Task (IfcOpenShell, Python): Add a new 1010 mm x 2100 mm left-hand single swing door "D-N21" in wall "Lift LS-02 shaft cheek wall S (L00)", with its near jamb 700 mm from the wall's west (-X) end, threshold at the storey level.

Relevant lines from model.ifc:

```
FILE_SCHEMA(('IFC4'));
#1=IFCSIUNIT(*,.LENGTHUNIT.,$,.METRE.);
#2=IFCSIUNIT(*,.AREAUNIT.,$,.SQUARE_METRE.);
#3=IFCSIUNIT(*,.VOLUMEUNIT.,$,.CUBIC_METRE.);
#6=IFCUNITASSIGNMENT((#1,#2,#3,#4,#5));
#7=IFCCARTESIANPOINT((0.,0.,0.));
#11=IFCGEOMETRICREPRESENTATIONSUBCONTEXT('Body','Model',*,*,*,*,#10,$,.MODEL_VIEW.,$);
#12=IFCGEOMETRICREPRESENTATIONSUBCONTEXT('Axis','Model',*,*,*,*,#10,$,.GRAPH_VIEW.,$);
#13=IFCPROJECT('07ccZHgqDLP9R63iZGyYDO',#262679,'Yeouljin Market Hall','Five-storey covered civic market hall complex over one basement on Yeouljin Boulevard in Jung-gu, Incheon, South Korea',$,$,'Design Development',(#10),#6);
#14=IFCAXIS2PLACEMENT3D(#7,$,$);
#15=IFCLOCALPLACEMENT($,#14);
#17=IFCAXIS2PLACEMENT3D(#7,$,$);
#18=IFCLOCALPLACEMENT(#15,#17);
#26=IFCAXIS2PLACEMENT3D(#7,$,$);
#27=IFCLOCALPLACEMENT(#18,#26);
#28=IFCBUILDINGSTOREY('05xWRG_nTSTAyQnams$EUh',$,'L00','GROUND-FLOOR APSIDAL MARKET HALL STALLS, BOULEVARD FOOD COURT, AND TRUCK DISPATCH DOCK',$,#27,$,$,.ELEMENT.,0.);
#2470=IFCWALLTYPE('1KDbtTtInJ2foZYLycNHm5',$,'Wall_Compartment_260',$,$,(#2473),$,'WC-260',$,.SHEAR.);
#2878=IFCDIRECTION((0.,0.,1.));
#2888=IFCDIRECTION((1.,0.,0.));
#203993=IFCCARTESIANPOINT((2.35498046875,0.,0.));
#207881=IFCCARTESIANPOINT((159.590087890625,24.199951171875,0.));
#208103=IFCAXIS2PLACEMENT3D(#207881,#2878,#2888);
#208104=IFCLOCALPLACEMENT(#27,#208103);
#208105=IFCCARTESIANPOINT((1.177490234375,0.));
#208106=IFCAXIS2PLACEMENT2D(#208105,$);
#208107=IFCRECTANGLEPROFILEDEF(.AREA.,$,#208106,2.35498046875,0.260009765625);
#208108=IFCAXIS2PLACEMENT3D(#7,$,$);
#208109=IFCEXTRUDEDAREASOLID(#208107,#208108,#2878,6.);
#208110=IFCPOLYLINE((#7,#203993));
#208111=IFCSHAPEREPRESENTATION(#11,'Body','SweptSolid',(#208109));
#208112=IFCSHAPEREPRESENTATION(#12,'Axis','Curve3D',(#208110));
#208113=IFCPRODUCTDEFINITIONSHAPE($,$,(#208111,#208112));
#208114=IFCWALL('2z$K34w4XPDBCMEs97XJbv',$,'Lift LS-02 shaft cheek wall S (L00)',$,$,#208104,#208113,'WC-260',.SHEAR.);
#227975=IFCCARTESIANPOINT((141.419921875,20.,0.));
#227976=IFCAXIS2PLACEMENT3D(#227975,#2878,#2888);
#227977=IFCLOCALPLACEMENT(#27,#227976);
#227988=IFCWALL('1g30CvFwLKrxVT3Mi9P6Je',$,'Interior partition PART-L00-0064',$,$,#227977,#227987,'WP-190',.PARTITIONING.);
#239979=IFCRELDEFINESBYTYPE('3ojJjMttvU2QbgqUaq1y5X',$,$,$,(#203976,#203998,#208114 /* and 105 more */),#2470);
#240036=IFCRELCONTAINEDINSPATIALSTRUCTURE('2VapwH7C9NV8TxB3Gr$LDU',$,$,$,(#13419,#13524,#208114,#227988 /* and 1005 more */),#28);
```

```python
import numpy as np
import ifcopenshell
import ifcopenshell.api.feature
import ifcopenshell.api.geometry
import ifcopenshell.api.root
import ifcopenshell.api.spatial
import ifcopenshell.geom
import ifcopenshell.util.element
import ifcopenshell.util.placement
import ifcopenshell.util.representation
import ifcopenshell.util.shape
import ifcopenshell.util.unit

model = ifcopenshell.open("model.ifc")
unit_scale = ifcopenshell.util.unit.calculate_unit_scale(model)
settings = ifcopenshell.geom.settings()


def volume(element):
    """Net volume in cubic metres, openings subtracted."""
    shape = ifcopenshell.geom.create_shape(settings, element)
    return ifcopenshell.util.shape.get_volume(shape.geometry)


wall = model.by_id(208114)
storey = ifcopenshell.util.element.get_container(wall, ifc_class="IfcBuildingStorey")
context = ifcopenshell.util.representation.get_context(model, "Model", "Body", "MODEL_VIEW")
before = volume(wall)

width, height, from_end, sill = 1.01, 2.1, 0.7, 0.0  # metres

# The wall runs along its own X axis, and the end named is its -X end.
wall_shape = ifcopenshell.geom.create_shape(settings, wall)
x, y, z = ifcopenshell.util.shape.get_vertices(wall_shape.geometry).T
start = x.min() + from_end
face, thickness = float(y.min()), float(y.max() - y.min())
wall_matrix = ifcopenshell.util.placement.get_local_placement(wall.ObjectPlacement)
level = ifcopenshell.util.placement.get_local_placement(storey.ObjectPlacement)[2, 3]


def in_wall(x, y):
    """Placement at x, y metres in the wall's axes, at sill height."""
    matrix = wall_matrix.copy()
    matrix[:, 3] = wall_matrix @ np.array([x / unit_scale, y / unit_scale, 0.0, 1.0])
    matrix[2, 3] = level + sill / unit_scale
    return matrix


# Opening: a box that overshoots both wall faces by 50 mm.
opening = ifcopenshell.api.root.create_entity(model, ifc_class="IfcOpeningElement", predefined_type="OPENING")
box = ifcopenshell.api.geometry.add_wall_representation(
    model, context=context, length=width, height=height, thickness=thickness + 0.1
)
ifcopenshell.api.geometry.assign_representation(model, product=opening, representation=box)
ifcopenshell.api.geometry.edit_object_placement(model, product=opening, matrix=in_wall(start, face - 0.05), is_si=False)
ifcopenshell.api.feature.add_feature(model, feature=opening, element=wall)

door = ifcopenshell.api.root.create_entity(model, ifc_class="IfcDoor", name="D-N21", predefined_type="DOOR")
door.OverallWidth, door.OverallHeight = width / unit_scale, height / unit_scale
door.OperationType = "SINGLE_SWING_LEFT"
body = ifcopenshell.api.geometry.add_door_representation(
    model,
    context=context,
    overall_width=door.OverallWidth,
    overall_height=door.OverallHeight,
    operation_type="SINGLE_SWING_LEFT",
    lining_properties={"LiningDepth": thickness / unit_scale, "ThresholdDepth": thickness / unit_scale},
)
ifcopenshell.api.geometry.assign_representation(model, product=door, representation=body)
ifcopenshell.api.spatial.assign_container(model, products=[door], relating_structure=storey)
ifcopenshell.api.feature.add_filling(model, opening=opening, element=door)

# The lining spans the wall, so the door starts at the wall face.
ifcopenshell.api.geometry.edit_object_placement(model, product=door, matrix=in_wall(start, face), is_si=False)

after = volume(wall)

print(f"wall volume {before:.3f} -> {after:.3f} m3")

model.write("model_v2.ifc")
```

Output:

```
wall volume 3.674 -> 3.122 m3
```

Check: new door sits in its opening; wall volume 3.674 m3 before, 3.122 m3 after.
